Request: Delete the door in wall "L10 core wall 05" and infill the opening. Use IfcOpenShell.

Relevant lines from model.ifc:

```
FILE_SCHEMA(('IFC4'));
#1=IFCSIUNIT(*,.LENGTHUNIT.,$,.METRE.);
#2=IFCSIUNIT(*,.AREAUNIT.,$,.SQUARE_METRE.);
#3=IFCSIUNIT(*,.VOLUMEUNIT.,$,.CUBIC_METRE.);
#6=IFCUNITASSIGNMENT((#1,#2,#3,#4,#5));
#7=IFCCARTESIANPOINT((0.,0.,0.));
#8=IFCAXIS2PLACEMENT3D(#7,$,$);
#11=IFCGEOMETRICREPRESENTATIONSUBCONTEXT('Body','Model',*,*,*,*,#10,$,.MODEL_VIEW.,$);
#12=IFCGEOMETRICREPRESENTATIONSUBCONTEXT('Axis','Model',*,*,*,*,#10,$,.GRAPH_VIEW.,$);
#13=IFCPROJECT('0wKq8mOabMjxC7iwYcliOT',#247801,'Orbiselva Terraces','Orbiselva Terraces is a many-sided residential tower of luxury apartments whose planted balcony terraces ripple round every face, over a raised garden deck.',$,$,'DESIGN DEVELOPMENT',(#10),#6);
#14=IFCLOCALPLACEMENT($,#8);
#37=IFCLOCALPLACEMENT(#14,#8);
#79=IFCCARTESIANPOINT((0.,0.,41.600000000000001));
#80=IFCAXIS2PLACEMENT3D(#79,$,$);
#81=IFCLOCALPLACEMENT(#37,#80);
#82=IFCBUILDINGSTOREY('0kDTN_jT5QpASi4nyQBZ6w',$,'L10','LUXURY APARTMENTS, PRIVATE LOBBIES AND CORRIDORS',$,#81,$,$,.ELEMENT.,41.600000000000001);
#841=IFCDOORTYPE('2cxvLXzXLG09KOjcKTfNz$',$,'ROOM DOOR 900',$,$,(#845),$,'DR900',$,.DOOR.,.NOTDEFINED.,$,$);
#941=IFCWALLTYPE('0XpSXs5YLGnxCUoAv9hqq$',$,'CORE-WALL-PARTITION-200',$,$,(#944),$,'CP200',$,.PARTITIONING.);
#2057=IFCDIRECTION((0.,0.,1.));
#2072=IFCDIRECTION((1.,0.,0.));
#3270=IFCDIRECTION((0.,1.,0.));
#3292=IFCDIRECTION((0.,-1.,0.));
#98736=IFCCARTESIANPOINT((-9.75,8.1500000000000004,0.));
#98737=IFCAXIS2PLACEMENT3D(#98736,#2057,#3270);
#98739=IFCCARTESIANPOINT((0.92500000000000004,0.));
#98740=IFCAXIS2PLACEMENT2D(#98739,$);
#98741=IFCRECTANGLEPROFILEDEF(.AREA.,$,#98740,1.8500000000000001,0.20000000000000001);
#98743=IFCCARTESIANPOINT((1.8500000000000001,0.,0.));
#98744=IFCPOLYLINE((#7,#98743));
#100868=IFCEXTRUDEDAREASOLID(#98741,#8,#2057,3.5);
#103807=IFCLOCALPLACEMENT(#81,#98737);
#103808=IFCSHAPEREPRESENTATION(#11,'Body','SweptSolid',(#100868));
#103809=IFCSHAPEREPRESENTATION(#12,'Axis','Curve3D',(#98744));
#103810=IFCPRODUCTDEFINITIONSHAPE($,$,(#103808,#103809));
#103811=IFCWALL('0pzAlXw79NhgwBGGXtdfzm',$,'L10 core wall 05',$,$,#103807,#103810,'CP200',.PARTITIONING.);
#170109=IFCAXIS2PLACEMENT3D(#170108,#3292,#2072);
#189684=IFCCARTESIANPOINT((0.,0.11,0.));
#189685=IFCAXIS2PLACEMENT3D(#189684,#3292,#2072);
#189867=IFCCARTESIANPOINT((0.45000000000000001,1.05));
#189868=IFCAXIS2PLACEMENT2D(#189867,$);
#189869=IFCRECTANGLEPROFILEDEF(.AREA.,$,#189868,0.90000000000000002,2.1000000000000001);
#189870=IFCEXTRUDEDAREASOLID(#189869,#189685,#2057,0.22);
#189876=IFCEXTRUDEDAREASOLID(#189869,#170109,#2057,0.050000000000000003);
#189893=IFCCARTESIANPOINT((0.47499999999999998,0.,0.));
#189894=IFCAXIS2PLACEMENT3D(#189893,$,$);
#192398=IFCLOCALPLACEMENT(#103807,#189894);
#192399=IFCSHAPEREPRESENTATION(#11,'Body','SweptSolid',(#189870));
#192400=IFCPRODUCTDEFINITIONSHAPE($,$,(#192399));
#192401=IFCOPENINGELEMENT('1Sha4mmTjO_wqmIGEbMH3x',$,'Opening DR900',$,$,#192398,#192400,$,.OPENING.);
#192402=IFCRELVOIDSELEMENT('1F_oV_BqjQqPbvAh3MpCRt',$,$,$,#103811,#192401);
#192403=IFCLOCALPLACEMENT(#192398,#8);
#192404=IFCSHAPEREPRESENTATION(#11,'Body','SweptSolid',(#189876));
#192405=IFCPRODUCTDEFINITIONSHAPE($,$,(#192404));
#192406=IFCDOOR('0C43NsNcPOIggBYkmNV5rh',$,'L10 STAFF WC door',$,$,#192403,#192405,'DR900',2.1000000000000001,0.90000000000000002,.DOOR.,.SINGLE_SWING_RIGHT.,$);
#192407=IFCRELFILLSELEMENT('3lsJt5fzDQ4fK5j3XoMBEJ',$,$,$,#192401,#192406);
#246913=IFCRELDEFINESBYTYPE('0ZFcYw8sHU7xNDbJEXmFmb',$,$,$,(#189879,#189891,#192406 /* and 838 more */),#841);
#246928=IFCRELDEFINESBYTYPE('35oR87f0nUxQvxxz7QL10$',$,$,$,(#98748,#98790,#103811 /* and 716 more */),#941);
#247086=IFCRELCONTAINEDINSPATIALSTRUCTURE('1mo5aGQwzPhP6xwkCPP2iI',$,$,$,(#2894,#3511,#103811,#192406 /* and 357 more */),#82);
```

```python
import ifcopenshell
import ifcopenshell.api.feature
import ifcopenshell.api.root
import ifcopenshell.geom
import ifcopenshell.util.shape

model = ifcopenshell.open("model.ifc")
settings = ifcopenshell.geom.settings()


def volume(element):
    """Net volume in cubic metres, openings subtracted."""
    shape = ifcopenshell.geom.create_shape(settings, element)
    return ifcopenshell.util.shape.get_volume(shape.geometry)


door = model.by_id(192406)
opening = door.FillsVoids[0].RelatingOpeningElement
wall = opening.VoidsElements[0].RelatingBuildingElement
before = volume(wall)

ifcopenshell.api.root.remove_product(model, product=door)
ifcopenshell.api.feature.remove_feature(model, feature=opening)

after = volume(wall)

print(f"wall volume {before:.3f} -> {after:.3f} m3")

model.write("model-out.ifc")
```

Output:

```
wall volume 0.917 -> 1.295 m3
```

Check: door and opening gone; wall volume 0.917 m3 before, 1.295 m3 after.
